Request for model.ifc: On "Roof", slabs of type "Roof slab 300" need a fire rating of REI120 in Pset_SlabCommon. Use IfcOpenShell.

First a look at what the model holds.

```python
import ifcopenshell
import ifcopenshell.util.element

model = ifcopenshell.open("model.ifc")
print(model.schema)
storey = next(s for s in model.by_type("IfcBuildingStorey") if s.Name == "Roof")
slabs = [e for e in ifcopenshell.util.element.get_decomposition(storey) if e.is_a("IfcSlab")]
seen = {}
for e in slabs:
    element_type = ifcopenshell.util.element.get_type(e)
    key = (element_type.Name if element_type != e and element_type else None, ifcopenshell.util.element.get_pset(e, "Pset_SlabCommon", "FireRating"))
    seen[key] = seen.get(key, 0) + 1
for (name, value), count in sorted(seen.items(), key=str):
    print(count, "x", name, "|", value)
```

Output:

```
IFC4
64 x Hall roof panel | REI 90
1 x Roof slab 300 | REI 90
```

```python
import ifcopenshell
import ifcopenshell.api.pset
import ifcopenshell.util.element

model = ifcopenshell.open("model.ifc")

storey = next(s for s in model.by_type("IfcBuildingStorey") if s.Name == "Roof")
slabs = [e for e in ifcopenshell.util.element.get_decomposition(storey) if e.is_a("IfcSlab")]

count = 0
for e in slabs:
    element_type = ifcopenshell.util.element.get_type(e)
    if element_type in (None, e) or element_type.Name != "Roof slab 300":
        continue
    # add_pset returns the element's existing set when there is one.
    pset = ifcopenshell.api.pset.add_pset(model, product=e, name="Pset_SlabCommon")
    ifcopenshell.api.pset.edit_pset(model, pset=pset, properties={"FireRating": "REI120"})
    count += 1

print(count, "slabs updated")

model.write("model_rev.ifc")
```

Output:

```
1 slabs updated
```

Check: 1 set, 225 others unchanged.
